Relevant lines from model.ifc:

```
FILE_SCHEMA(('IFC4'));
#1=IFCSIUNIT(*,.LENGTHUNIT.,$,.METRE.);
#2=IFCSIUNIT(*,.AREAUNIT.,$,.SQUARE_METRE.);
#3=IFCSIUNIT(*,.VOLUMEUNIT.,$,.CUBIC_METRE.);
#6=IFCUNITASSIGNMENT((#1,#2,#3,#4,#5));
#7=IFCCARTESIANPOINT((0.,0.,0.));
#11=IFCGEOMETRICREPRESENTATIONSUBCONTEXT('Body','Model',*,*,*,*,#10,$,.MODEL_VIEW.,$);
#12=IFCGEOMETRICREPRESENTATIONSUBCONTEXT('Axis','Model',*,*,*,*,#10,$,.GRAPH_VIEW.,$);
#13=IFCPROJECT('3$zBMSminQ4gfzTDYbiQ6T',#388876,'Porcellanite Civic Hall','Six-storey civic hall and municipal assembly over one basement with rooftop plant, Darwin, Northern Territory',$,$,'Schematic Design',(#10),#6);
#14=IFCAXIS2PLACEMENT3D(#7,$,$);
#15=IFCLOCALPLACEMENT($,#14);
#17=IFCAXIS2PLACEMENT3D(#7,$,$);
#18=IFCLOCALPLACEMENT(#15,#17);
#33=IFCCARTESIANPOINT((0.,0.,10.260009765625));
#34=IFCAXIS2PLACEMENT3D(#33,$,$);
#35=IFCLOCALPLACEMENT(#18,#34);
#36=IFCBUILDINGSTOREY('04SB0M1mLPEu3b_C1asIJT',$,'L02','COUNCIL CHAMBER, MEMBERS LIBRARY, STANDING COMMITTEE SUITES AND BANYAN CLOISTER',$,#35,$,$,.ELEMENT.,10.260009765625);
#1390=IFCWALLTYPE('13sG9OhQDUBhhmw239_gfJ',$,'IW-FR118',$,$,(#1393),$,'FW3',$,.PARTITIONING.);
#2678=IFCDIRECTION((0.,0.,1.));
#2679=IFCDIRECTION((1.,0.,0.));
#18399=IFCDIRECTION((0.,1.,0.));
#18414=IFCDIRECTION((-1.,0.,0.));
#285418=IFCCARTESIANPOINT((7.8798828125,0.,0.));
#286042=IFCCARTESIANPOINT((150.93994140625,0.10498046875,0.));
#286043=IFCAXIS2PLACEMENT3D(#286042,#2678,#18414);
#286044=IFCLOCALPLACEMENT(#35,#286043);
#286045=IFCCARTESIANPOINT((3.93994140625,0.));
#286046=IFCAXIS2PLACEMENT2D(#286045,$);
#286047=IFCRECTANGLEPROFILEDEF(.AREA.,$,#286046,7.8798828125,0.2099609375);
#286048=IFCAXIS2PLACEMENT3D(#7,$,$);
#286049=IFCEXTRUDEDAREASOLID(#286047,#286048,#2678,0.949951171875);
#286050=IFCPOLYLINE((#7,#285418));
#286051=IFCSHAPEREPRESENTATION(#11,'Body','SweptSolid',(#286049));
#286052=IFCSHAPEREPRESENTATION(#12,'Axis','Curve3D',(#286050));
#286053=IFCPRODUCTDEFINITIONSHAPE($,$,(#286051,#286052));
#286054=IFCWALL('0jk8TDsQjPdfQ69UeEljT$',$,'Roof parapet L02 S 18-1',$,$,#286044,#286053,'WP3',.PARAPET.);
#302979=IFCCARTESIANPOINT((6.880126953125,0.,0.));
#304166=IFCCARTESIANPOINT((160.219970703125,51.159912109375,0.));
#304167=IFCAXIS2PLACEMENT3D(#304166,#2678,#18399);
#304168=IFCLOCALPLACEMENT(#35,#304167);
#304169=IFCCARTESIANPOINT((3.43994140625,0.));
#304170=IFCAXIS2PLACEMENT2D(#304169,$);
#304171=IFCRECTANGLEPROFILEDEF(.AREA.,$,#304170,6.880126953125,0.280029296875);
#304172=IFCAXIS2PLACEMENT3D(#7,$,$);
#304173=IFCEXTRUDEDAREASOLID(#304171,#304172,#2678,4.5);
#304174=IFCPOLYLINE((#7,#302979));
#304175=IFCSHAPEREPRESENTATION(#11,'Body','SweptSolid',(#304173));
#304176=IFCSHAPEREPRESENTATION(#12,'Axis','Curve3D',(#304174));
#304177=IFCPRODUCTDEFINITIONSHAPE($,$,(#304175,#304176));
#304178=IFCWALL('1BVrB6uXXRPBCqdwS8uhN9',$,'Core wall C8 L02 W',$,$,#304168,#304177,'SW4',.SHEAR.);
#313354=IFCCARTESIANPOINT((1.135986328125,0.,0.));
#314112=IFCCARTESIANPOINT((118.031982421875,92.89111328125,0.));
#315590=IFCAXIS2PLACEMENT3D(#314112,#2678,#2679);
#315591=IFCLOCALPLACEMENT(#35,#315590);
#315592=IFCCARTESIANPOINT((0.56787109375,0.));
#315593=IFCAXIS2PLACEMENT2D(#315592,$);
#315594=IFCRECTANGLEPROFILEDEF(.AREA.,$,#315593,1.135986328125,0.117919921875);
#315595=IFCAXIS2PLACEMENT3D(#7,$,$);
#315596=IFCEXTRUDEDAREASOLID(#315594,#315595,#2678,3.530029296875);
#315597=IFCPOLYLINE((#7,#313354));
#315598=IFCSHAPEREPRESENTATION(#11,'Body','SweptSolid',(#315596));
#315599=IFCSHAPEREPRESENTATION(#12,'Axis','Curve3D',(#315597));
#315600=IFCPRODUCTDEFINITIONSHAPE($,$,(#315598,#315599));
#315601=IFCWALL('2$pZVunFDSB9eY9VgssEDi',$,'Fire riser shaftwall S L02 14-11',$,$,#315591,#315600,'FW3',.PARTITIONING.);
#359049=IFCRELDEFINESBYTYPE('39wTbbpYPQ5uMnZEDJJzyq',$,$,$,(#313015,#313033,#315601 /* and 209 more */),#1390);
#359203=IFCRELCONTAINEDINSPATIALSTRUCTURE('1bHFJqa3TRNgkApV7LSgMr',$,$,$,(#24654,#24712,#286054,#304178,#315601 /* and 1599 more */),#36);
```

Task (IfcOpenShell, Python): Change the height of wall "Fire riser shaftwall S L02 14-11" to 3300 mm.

```python
import ifcopenshell
import ifcopenshell.geom
import ifcopenshell.util.representation
import ifcopenshell.util.shape
import ifcopenshell.util.unit

model = ifcopenshell.open("model.ifc")
unit_scale = ifcopenshell.util.unit.calculate_unit_scale(model)
settings = ifcopenshell.geom.settings()


def volume(element):
    """Net volume in cubic metres, openings subtracted."""
    shape = ifcopenshell.geom.create_shape(settings, element)
    return ifcopenshell.util.shape.get_volume(shape.geometry)


wall = model.by_id(315601)
before = volume(wall)

body = ifcopenshell.util.representation.get_representation(wall, "Model", "Body")
solid = body.Items[0]
old_height = solid.Depth
solid.Depth = 3.3 / unit_scale
after = volume(wall)

print(f"height {old_height:g} -> {solid.Depth:g}, volume {before:.3f} -> {after:.3f} m3")

model.write("model_updated.ifc")
```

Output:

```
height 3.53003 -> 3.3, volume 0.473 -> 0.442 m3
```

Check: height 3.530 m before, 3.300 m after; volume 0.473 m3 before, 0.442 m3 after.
